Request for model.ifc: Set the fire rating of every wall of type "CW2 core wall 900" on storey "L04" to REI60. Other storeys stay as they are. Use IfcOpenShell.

First a look at what the model holds.

```python
import ifcopenshell
import ifcopenshell.util.element

model = ifcopenshell.open("model.ifc")
print(model.schema)
storey = next(s for s in model.by_type("IfcBuildingStorey") if s.Name == "L04")
walls = [e for e in ifcopenshell.util.element.get_decomposition(storey) if e.is_a("IfcWall")]
seen = {}
for e in walls:
    element_type = ifcopenshell.util.element.get_type(e)
    key = (element_type.Name if element_type != e and element_type else None, ifcopenshell.util.element.get_pset(e, "Pset_WallCommon", "FireRating"))
    seen[key] = seen.get(key, 0) + 1
for (name, value), count in sorted(seen.items(), key=str):
    print(count, "x", name, "|", value)
```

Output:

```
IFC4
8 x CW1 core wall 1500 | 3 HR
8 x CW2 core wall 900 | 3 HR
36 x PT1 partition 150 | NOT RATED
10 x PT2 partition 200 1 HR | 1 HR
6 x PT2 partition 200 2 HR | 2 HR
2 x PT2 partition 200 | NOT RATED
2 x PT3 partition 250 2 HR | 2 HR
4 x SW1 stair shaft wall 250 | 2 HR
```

```python
import ifcopenshell
import ifcopenshell.api.pset
import ifcopenshell.util.element

model = ifcopenshell.open("model.ifc")

storey = next(s for s in model.by_type("IfcBuildingStorey") if s.Name == "L04")
walls = [e for e in ifcopenshell.util.element.get_decomposition(storey) if e.is_a("IfcWall")]

count = 0
for e in walls:
    element_type = ifcopenshell.util.element.get_type(e)
    if element_type in (None, e) or element_type.Name != "CW2 core wall 900":
        continue
    found = ifcopenshell.util.element.get_pset(e, "Pset_WallCommon", should_inherit=False)
    if found:
        pset = model.by_id(found["id"])
        if len(ifcopenshell.util.element.get_elements_by_pset(pset)) > 1:
            pset = ifcopenshell.api.pset.unshare_pset(model, products=[e], pset=pset)[0]
    else:
        pset = ifcopenshell.api.pset.add_pset(model, product=e, name="Pset_WallCommon")
    ifcopenshell.api.pset.edit_pset(model, pset=pset, properties={"FireRating": "REI60"})
    count += 1

print(count, "walls updated")

model.write("model-out.ifc")
```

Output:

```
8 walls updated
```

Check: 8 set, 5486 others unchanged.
